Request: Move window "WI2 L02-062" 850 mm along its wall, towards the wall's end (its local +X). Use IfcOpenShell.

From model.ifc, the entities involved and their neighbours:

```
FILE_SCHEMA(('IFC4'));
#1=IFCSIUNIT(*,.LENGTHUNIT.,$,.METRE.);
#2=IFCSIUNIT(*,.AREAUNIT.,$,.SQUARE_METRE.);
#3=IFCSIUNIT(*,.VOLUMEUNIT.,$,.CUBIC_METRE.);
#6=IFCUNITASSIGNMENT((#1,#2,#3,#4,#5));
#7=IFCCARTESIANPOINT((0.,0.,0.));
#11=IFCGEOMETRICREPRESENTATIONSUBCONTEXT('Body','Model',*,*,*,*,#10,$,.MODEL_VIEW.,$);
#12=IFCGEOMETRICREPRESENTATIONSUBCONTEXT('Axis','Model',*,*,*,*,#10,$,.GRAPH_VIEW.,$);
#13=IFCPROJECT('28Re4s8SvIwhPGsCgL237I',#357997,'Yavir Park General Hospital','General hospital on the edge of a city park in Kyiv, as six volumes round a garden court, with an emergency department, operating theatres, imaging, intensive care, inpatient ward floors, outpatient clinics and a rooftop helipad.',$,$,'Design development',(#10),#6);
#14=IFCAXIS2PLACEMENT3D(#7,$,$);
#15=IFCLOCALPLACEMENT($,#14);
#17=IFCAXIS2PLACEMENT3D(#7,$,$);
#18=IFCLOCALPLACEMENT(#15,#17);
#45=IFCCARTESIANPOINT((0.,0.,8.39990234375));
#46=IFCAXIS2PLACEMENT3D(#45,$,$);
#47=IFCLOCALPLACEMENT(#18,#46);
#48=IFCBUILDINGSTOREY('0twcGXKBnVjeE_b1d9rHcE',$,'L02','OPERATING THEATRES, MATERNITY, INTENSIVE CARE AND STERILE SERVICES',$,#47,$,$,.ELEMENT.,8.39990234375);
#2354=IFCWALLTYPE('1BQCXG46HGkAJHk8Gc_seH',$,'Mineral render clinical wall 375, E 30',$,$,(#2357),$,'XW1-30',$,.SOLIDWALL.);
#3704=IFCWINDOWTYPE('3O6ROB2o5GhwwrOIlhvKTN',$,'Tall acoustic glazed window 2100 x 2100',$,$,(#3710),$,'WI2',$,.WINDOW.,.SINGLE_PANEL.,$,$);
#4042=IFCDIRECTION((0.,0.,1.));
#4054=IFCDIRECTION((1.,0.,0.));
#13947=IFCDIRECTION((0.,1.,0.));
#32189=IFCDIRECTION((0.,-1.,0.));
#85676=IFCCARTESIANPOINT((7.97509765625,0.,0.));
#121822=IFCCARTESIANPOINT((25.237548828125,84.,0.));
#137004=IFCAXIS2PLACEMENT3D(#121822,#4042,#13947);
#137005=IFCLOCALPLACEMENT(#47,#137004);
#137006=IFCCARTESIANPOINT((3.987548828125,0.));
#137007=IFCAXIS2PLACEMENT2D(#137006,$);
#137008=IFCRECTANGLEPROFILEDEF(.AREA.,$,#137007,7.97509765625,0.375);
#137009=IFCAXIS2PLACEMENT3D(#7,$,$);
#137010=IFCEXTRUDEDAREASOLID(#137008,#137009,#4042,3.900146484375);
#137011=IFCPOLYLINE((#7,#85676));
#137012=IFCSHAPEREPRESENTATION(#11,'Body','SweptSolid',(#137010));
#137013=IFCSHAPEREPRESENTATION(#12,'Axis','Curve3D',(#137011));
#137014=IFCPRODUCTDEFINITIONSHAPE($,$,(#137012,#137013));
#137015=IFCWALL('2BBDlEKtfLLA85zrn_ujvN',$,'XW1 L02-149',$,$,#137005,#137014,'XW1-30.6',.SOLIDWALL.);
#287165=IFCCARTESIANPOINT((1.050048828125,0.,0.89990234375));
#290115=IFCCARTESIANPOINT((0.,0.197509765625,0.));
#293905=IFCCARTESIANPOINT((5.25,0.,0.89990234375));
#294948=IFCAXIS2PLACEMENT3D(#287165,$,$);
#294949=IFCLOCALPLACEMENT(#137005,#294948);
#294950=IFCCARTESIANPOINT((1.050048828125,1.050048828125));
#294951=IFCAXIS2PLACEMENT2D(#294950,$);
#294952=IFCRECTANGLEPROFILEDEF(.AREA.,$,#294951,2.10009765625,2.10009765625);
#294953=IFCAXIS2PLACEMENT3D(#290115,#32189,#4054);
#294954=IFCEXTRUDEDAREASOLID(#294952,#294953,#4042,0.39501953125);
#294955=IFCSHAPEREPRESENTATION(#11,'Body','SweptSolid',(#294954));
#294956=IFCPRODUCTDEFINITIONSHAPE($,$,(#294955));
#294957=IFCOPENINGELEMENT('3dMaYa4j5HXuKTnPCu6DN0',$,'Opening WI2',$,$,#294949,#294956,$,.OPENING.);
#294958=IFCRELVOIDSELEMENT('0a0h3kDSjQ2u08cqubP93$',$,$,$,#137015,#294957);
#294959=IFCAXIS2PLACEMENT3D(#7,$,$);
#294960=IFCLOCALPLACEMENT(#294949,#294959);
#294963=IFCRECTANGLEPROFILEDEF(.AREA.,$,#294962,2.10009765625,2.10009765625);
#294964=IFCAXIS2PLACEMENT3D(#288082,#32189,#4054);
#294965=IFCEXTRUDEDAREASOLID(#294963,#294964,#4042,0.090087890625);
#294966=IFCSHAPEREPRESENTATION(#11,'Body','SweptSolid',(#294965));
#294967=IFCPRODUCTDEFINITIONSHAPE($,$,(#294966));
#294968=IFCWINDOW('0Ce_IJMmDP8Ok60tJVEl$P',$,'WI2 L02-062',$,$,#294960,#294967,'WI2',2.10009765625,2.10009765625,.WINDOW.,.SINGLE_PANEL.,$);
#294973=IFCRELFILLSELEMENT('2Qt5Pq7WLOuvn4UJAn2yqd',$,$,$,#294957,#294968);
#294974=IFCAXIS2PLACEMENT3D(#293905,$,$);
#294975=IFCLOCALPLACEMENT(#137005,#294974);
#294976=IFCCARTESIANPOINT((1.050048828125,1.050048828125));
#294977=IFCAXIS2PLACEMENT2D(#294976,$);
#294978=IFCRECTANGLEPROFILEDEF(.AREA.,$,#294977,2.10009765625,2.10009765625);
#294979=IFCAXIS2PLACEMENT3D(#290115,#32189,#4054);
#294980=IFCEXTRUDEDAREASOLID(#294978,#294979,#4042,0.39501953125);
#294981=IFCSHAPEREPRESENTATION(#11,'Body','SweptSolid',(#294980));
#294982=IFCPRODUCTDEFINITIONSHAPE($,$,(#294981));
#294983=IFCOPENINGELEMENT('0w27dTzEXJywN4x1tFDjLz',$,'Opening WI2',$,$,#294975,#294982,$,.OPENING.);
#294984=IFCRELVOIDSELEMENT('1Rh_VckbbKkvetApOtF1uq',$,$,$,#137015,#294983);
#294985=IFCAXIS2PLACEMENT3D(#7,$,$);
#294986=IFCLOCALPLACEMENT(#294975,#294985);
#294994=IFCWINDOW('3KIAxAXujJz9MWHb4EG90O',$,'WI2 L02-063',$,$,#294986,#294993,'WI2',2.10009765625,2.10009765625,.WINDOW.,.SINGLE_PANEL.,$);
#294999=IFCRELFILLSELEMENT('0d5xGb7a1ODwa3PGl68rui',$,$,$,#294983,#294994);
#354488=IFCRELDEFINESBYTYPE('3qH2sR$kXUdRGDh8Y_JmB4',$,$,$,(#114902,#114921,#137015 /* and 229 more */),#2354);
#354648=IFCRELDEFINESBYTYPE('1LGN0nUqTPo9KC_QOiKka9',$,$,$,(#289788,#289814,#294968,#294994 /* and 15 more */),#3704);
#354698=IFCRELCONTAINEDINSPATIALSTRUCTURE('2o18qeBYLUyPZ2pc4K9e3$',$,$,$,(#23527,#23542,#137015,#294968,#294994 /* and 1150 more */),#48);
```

```python
import ifcopenshell
import ifcopenshell.api.geometry
import ifcopenshell.util.placement

model = ifcopenshell.open("model.ifc")

window = model.by_guid("0Ce_IJMmDP8Ok60tJVEl$P")
opening = window.FillsVoids[0].RelatingOpeningElement
wall = opening.VoidsElements[0].RelatingBuildingElement

wall_matrix = ifcopenshell.util.placement.get_local_placement(wall.ObjectPlacement)
shift = wall_matrix[:3, 0] * 0.85
before = ifcopenshell.util.placement.get_local_placement(window.ObjectPlacement)[:3, 3].copy()

# The window is placed relative to its opening, so it follows when the opening moves.
matrix = ifcopenshell.util.placement.get_local_placement(opening.ObjectPlacement)
matrix[:3, 3] += shift
ifcopenshell.api.geometry.edit_object_placement(
    model, product=opening, matrix=matrix, is_si=False, should_transform_children=True
)

after = ifcopenshell.util.placement.get_local_placement(window.ObjectPlacement)[:3, 3]
print("window moved by", (after - before).round(3) + 0.0)

model.write("model-out.ifc")
```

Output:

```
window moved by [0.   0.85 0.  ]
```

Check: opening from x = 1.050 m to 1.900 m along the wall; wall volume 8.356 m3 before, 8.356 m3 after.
